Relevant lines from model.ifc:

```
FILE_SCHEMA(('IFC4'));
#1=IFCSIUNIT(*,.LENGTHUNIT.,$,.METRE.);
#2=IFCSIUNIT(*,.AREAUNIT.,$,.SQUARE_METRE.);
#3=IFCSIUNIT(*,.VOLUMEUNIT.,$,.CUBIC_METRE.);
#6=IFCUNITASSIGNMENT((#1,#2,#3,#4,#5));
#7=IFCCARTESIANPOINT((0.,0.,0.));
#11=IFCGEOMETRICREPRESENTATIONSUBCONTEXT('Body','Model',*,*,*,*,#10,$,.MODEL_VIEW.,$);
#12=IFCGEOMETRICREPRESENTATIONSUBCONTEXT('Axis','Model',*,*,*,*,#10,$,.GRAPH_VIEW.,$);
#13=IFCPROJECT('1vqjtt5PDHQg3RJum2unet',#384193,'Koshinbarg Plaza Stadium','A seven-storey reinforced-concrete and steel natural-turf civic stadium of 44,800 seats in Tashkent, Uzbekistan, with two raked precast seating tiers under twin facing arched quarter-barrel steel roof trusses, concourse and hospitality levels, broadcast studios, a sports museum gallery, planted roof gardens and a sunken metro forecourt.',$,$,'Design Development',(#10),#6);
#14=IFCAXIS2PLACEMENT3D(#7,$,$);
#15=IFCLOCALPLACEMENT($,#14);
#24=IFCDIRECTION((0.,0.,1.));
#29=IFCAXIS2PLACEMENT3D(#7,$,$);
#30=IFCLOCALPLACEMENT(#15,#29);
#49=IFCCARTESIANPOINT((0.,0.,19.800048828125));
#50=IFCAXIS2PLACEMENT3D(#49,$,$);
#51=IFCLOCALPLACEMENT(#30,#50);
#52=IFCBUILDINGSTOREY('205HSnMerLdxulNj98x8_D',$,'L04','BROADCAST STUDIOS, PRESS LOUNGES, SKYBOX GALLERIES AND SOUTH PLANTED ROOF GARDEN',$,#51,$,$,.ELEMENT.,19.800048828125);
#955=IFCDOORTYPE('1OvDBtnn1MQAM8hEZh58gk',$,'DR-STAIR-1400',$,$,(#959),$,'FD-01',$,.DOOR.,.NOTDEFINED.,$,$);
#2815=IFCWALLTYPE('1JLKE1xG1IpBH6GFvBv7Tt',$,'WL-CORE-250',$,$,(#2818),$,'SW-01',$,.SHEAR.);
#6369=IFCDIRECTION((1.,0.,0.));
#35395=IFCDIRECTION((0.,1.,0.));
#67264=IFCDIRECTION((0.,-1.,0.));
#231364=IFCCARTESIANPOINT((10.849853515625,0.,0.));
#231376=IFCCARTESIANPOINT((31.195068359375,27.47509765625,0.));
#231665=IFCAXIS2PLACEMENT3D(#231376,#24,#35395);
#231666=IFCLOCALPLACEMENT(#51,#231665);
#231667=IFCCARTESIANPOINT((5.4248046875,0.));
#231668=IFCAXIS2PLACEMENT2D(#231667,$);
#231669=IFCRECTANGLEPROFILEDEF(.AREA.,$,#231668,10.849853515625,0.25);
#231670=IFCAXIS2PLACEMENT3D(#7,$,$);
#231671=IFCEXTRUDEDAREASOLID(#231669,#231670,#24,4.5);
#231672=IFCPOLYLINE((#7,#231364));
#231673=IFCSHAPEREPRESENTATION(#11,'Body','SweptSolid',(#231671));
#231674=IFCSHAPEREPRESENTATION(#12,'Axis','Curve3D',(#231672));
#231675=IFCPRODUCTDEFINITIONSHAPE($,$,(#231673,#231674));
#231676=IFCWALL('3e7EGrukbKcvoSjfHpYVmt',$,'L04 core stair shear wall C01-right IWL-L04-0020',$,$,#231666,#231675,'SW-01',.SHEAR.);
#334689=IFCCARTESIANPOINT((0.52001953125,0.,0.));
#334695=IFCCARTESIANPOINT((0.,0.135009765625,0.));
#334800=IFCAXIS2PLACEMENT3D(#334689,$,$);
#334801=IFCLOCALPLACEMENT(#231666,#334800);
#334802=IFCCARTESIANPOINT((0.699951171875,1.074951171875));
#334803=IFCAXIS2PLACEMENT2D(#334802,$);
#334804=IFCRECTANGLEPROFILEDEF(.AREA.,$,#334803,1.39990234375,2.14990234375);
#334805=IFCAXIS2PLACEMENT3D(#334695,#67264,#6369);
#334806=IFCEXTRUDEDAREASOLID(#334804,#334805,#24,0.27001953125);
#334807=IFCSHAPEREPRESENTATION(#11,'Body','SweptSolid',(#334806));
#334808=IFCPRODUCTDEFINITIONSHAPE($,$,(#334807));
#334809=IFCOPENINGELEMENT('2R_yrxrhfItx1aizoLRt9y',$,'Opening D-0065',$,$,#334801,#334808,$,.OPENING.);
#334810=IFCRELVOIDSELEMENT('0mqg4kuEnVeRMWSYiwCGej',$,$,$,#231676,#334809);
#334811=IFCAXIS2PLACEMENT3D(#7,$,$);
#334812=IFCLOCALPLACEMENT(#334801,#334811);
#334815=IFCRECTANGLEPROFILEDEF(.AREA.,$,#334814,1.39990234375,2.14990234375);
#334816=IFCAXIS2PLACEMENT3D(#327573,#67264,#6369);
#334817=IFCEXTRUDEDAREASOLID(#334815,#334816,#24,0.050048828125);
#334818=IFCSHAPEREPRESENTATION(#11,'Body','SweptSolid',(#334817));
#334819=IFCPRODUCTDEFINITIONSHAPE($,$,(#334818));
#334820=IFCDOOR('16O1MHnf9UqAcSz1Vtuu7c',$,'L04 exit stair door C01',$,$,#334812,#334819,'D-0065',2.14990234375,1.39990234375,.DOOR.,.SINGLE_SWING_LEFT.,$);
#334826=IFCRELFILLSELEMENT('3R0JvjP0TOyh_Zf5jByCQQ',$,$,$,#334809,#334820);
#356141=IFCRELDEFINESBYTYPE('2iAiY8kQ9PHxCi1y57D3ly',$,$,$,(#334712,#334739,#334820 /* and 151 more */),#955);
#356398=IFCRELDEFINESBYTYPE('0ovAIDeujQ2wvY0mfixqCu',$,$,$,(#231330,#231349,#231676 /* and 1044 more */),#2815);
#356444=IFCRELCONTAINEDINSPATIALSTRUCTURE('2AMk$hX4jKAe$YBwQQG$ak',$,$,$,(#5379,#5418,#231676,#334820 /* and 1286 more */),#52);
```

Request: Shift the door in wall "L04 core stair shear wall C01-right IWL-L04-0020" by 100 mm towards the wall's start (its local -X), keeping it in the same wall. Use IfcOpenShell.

```python
import ifcopenshell
import ifcopenshell.api.geometry
import ifcopenshell.util.placement
import ifcopenshell.util.unit

model = ifcopenshell.open("model.ifc")
unit_scale = ifcopenshell.util.unit.calculate_unit_scale(model)

door = model.by_guid("16O1MHnf9UqAcSz1Vtuu7c")
opening = door.FillsVoids[0].RelatingOpeningElement
wall = opening.VoidsElements[0].RelatingBuildingElement

wall_matrix = ifcopenshell.util.placement.get_local_placement(wall.ObjectPlacement)
shift = wall_matrix[:3, 0] * -0.1 / unit_scale
before = ifcopenshell.util.placement.get_local_placement(door.ObjectPlacement)[:3, 3].copy()

# The door is placed relative to its opening, so it follows when the opening moves.
matrix = ifcopenshell.util.placement.get_local_placement(opening.ObjectPlacement)
matrix[:3, 3] += shift
ifcopenshell.api.geometry.edit_object_placement(
    model, product=opening, matrix=matrix, is_si=False, should_transform_children=True
)

after = ifcopenshell.util.placement.get_local_placement(door.ObjectPlacement)[:3, 3]
print("door moved by", (after - before).round(3) + 0.0)

model.write("model_v2.ifc")
```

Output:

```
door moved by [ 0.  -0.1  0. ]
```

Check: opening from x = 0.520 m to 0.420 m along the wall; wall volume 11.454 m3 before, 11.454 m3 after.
